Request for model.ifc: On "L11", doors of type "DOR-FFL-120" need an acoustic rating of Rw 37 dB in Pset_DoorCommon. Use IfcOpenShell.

First a look at what the model holds.

```python
import ifcopenshell
import ifcopenshell.util.element

model = ifcopenshell.open("model.ifc")
print(model.schema)
storey = next(s for s in model.by_type("IfcBuildingStorey") if s.Name == "L11")
doors = [e for e in ifcopenshell.util.element.get_decomposition(storey) if e.is_a("IfcDoor")]
seen = {}
for e in doors:
    element_type = ifcopenshell.util.element.get_type(e)
    key = (element_type.Name if element_type != e and element_type else None, ifcopenshell.util.element.get_pset(e, "Pset_DoorCommon", "AcousticRating"))
    seen[key] = seen.get(key, 0) + 1
for (name, value), count in sorted(seen.items(), key=str):
    print(count, "x", name, "|", value)
```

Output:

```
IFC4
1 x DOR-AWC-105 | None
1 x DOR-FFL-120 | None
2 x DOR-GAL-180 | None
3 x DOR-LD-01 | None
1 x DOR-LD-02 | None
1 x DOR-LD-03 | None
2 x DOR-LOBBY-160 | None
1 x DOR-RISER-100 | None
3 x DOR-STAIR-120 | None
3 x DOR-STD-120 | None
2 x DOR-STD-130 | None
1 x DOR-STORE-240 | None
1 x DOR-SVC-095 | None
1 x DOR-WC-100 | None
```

```python
import ifcopenshell
import ifcopenshell.api.pset
import ifcopenshell.util.element

model = ifcopenshell.open("model.ifc")

storey = next(s for s in model.by_type("IfcBuildingStorey") if s.Name == "L11")
doors = [e for e in ifcopenshell.util.element.get_decomposition(storey) if e.is_a("IfcDoor")]

count = 0
for e in doors:
    element_type = ifcopenshell.util.element.get_type(e)
    if element_type in (None, e) or element_type.Name != "DOR-FFL-120":
        continue
    # add_pset returns the element's existing set when there is one.
    pset = ifcopenshell.api.pset.add_pset(model, product=e, name="Pset_DoorCommon")
    ifcopenshell.api.pset.edit_pset(model, pset=pset, properties={"AcousticRating": "Rw 37 dB"})
    count += 1

print(count, "doors updated")

model.write("model_updated.ifc")
```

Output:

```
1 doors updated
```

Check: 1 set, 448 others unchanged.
